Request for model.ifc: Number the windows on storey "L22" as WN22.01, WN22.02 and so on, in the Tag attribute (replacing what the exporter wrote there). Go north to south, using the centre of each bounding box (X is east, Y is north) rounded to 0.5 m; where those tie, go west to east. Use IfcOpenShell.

First a look at what the model holds.

```python
import ifcopenshell
import ifcopenshell.util.element
import ifcopenshell.util.placement

model = ifcopenshell.open("model.ifc")
print(model.schema)
storey = next(s for s in model.by_type("IfcBuildingStorey") if s.Name == "L22")
windows = [e for e in ifcopenshell.util.element.get_decomposition(storey) if e.is_a("IfcWindow")]
for e in sorted(windows, key=lambda e: e.id()):
    origin = ifcopenshell.util.placement.get_local_placement(e.ObjectPlacement)[:3, 3]
    print(e.id(), e.Tag, e.Name, origin.round(2) + 0.0, sep=" | ")
```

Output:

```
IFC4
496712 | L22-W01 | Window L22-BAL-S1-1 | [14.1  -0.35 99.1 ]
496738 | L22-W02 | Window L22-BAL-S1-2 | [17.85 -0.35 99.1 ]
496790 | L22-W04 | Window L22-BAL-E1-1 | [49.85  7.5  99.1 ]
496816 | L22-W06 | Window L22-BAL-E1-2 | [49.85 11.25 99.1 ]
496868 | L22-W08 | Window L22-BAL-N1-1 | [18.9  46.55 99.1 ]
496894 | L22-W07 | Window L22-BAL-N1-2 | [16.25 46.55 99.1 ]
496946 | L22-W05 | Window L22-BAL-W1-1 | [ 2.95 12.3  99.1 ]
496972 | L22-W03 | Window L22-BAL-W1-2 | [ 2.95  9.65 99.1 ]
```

```python
import ifcopenshell
import ifcopenshell.geom
import ifcopenshell.util.element
import ifcopenshell.util.shape

model = ifcopenshell.open("model.ifc")
settings = ifcopenshell.geom.settings()
settings.set("use-world-coords", True)


def centre(element):
    shape = ifcopenshell.geom.create_shape(settings, element)
    return ifcopenshell.util.shape.get_bbox_centroid(shape.geometry)


storey = next(s for s in model.by_type("IfcBuildingStorey") if s.Name == "L22")
windows = [e for e in ifcopenshell.util.element.get_decomposition(storey) if e.is_a("IfcWindow")]

# Insertion points can sit at a corner or the storey origin, so sort by the geometry (in metres).
centres = {e: centre(e) for e in windows}
windows.sort(key=lambda e: (-round(centres[e][1] / 0.5), centres[e][0]))

for i, e in enumerate(windows, start=1):
    number = f"WN22.{i:02d}"
    e.Tag = number
    print(e.id(), number)

model.write("model_rev.ifc")
```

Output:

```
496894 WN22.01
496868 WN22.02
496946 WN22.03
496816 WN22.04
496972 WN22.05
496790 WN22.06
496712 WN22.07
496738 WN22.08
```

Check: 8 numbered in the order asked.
